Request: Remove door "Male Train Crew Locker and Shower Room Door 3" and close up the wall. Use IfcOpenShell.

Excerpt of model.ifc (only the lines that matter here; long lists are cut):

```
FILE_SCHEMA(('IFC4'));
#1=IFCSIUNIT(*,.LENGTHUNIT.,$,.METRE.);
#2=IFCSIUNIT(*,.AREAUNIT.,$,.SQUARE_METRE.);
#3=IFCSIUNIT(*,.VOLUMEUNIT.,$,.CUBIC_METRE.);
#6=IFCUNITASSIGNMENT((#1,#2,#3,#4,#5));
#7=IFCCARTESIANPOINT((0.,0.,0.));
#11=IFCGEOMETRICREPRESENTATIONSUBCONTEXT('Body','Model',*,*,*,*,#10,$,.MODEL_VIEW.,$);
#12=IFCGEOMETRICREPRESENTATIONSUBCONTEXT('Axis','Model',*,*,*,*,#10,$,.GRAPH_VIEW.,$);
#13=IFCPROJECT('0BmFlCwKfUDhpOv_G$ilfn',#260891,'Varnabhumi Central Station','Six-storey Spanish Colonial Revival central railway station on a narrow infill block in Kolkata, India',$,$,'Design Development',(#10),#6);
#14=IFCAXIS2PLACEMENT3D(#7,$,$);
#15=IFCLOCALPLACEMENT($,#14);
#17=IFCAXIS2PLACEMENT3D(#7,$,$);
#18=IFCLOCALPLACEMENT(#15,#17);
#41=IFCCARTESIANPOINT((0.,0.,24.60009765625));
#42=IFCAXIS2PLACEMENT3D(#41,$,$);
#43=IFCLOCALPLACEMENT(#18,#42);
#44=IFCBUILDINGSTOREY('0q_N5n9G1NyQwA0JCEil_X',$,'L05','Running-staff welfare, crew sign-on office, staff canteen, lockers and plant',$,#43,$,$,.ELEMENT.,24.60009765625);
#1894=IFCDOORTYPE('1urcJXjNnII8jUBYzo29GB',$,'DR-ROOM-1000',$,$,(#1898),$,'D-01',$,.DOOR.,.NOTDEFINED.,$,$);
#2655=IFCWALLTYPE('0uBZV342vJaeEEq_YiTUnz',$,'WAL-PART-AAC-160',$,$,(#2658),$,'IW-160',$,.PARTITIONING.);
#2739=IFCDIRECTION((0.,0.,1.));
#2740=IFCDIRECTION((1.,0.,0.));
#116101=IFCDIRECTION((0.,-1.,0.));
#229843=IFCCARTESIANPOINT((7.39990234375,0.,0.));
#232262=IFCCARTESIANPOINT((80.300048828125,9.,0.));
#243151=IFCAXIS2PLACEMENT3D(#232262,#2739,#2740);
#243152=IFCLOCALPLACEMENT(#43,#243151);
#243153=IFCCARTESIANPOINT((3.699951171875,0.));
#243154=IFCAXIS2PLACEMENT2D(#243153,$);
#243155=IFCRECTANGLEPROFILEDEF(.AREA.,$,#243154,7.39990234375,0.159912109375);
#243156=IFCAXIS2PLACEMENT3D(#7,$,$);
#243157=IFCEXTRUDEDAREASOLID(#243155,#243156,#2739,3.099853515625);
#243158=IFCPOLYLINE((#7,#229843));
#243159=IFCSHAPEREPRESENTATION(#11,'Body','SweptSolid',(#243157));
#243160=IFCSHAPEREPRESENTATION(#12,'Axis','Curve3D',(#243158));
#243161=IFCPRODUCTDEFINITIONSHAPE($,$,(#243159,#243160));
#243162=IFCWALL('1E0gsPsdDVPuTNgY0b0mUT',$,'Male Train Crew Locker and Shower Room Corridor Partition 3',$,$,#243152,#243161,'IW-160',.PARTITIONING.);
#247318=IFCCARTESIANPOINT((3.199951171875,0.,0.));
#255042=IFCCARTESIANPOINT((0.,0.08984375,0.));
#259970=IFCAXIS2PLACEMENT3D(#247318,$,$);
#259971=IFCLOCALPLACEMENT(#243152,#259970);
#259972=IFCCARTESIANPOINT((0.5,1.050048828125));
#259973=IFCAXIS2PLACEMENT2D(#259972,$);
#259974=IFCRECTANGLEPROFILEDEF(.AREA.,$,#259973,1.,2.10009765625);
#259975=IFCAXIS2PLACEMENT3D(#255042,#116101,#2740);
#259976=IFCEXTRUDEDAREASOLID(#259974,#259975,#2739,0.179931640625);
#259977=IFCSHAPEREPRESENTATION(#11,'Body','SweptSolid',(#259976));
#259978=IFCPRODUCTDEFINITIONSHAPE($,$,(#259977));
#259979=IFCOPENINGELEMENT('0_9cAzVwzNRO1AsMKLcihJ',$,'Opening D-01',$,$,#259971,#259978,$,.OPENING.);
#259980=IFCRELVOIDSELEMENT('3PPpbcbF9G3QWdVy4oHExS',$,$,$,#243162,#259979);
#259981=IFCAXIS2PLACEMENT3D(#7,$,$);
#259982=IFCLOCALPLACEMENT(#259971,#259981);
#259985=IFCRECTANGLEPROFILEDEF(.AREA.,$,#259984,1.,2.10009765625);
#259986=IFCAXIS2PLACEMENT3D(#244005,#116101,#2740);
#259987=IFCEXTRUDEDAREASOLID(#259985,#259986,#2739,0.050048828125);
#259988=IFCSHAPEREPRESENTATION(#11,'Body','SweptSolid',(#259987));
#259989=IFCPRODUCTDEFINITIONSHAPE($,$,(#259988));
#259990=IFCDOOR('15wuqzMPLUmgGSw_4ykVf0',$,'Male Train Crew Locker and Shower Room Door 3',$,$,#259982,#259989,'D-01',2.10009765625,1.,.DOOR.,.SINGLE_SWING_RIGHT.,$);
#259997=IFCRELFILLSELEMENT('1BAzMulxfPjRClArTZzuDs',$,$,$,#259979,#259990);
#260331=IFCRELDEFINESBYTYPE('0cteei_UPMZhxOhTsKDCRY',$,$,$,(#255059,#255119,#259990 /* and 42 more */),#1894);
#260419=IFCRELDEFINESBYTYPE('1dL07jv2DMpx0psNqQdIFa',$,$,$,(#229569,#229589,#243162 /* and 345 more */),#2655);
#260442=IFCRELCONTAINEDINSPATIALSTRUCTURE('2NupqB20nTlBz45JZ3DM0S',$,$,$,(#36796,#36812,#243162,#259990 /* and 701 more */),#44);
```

```python
import ifcopenshell
import ifcopenshell.api.feature
import ifcopenshell.api.root
import ifcopenshell.geom
import ifcopenshell.util.shape

model = ifcopenshell.open("model.ifc")
settings = ifcopenshell.geom.settings()


def volume(element):
    """Net volume in cubic metres, openings subtracted."""
    shape = ifcopenshell.geom.create_shape(settings, element)
    return ifcopenshell.util.shape.get_volume(shape.geometry)


door = model.by_id(259990)
opening = door.FillsVoids[0].RelatingOpeningElement
wall = opening.VoidsElements[0].RelatingBuildingElement
before = volume(wall)

ifcopenshell.api.root.remove_product(model, product=door)
ifcopenshell.api.feature.remove_feature(model, feature=opening)

after = volume(wall)

print(f"wall volume {before:.3f} -> {after:.3f} m3")

model.write("model_v2.ifc")
```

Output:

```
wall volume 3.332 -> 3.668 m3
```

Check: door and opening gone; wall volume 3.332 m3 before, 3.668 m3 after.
